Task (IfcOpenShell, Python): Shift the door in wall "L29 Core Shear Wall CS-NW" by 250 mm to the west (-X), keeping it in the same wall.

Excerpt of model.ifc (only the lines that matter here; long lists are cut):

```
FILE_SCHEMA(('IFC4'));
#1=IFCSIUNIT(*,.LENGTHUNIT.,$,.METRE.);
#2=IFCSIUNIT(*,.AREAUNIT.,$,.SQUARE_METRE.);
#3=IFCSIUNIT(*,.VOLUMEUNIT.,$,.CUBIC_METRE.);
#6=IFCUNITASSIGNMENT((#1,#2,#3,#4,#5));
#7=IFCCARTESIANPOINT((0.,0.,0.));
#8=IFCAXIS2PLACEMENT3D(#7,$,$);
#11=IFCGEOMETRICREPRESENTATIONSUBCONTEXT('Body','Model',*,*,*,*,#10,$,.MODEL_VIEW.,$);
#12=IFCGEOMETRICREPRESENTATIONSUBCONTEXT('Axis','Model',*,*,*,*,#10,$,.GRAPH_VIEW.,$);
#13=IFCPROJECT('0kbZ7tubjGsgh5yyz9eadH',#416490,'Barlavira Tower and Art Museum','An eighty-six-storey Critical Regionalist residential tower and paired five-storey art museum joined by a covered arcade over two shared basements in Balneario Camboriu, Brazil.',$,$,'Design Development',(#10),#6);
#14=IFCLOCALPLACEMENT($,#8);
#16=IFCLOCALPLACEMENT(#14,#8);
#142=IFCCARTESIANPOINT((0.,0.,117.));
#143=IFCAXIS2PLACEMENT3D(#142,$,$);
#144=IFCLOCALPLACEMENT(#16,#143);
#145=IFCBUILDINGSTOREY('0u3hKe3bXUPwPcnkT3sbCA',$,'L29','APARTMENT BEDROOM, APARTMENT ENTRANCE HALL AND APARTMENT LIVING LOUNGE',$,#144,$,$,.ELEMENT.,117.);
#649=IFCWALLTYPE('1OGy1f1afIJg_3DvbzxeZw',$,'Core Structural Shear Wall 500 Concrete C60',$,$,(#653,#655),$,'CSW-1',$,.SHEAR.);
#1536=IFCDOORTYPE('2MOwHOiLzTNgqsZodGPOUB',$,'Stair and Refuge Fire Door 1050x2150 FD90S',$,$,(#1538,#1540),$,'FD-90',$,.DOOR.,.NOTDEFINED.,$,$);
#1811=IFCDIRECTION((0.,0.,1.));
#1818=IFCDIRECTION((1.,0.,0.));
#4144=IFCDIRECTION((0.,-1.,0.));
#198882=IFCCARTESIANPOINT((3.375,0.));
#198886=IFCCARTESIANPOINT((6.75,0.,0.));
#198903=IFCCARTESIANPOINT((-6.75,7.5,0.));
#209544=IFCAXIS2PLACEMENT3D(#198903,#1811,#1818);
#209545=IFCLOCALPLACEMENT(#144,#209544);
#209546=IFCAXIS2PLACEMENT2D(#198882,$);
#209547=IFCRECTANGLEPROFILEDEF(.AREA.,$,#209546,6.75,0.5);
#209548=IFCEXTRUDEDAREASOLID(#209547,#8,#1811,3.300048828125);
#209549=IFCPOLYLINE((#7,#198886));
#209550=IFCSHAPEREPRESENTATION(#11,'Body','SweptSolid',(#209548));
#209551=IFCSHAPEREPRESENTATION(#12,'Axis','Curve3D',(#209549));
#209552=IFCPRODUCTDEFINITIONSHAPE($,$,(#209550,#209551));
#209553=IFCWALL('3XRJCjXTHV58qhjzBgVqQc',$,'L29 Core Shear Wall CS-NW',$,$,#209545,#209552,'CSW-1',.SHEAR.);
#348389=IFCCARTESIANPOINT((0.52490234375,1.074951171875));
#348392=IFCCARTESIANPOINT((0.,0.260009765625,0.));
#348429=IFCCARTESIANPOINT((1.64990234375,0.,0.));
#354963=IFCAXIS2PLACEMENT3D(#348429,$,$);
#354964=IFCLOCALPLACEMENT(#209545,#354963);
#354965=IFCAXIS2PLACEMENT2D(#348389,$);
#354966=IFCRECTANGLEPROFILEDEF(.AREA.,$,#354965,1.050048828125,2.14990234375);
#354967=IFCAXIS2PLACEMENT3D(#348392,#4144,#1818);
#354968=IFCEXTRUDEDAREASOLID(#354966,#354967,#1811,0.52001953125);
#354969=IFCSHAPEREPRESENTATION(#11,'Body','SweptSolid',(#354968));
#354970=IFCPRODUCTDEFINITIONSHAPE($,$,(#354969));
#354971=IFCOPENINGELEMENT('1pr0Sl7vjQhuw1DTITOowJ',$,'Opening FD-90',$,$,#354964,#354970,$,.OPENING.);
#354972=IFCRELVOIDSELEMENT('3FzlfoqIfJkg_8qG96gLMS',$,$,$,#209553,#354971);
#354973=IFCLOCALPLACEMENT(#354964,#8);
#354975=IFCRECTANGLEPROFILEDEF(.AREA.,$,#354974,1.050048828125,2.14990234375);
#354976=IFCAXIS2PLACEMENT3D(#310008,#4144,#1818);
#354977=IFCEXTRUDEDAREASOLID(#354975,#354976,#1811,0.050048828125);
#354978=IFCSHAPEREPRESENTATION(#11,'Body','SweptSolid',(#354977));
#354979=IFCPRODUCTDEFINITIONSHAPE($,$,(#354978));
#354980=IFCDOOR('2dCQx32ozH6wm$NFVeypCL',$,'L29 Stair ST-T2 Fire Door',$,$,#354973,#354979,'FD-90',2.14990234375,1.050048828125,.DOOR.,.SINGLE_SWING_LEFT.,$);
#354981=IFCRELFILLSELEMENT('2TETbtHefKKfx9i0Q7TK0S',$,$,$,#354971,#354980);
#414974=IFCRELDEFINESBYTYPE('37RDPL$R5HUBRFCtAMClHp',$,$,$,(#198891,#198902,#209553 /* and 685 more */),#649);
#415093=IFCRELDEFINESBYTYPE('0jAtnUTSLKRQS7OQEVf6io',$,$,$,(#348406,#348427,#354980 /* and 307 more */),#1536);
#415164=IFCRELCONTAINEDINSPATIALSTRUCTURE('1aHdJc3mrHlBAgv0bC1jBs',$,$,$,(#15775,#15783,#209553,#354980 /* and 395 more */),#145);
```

```python
import ifcopenshell
import ifcopenshell.api.geometry
import ifcopenshell.util.placement
import ifcopenshell.util.unit

model = ifcopenshell.open("model.ifc")
unit_scale = ifcopenshell.util.unit.calculate_unit_scale(model)

door = model.by_id(354980)
opening = door.FillsVoids[0].RelatingOpeningElement
wall = opening.VoidsElements[0].RelatingBuildingElement

wall_matrix = ifcopenshell.util.placement.get_local_placement(wall.ObjectPlacement)
shift = wall_matrix[:3, 0] * -0.25 / unit_scale
before = ifcopenshell.util.placement.get_local_placement(door.ObjectPlacement)[:3, 3].copy()

# The door is placed relative to its opening, so it follows when the opening moves.
matrix = ifcopenshell.util.placement.get_local_placement(opening.ObjectPlacement)
matrix[:3, 3] += shift
ifcopenshell.api.geometry.edit_object_placement(
    model, product=opening, matrix=matrix, is_si=False, should_transform_children=True
)

after = ifcopenshell.util.placement.get_local_placement(door.ObjectPlacement)[:3, 3]
print("door moved by", (after - before).round(3) + 0.0)

model.write("model_rev.ifc")
```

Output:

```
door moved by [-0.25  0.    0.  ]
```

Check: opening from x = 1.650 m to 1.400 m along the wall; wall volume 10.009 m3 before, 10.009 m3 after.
